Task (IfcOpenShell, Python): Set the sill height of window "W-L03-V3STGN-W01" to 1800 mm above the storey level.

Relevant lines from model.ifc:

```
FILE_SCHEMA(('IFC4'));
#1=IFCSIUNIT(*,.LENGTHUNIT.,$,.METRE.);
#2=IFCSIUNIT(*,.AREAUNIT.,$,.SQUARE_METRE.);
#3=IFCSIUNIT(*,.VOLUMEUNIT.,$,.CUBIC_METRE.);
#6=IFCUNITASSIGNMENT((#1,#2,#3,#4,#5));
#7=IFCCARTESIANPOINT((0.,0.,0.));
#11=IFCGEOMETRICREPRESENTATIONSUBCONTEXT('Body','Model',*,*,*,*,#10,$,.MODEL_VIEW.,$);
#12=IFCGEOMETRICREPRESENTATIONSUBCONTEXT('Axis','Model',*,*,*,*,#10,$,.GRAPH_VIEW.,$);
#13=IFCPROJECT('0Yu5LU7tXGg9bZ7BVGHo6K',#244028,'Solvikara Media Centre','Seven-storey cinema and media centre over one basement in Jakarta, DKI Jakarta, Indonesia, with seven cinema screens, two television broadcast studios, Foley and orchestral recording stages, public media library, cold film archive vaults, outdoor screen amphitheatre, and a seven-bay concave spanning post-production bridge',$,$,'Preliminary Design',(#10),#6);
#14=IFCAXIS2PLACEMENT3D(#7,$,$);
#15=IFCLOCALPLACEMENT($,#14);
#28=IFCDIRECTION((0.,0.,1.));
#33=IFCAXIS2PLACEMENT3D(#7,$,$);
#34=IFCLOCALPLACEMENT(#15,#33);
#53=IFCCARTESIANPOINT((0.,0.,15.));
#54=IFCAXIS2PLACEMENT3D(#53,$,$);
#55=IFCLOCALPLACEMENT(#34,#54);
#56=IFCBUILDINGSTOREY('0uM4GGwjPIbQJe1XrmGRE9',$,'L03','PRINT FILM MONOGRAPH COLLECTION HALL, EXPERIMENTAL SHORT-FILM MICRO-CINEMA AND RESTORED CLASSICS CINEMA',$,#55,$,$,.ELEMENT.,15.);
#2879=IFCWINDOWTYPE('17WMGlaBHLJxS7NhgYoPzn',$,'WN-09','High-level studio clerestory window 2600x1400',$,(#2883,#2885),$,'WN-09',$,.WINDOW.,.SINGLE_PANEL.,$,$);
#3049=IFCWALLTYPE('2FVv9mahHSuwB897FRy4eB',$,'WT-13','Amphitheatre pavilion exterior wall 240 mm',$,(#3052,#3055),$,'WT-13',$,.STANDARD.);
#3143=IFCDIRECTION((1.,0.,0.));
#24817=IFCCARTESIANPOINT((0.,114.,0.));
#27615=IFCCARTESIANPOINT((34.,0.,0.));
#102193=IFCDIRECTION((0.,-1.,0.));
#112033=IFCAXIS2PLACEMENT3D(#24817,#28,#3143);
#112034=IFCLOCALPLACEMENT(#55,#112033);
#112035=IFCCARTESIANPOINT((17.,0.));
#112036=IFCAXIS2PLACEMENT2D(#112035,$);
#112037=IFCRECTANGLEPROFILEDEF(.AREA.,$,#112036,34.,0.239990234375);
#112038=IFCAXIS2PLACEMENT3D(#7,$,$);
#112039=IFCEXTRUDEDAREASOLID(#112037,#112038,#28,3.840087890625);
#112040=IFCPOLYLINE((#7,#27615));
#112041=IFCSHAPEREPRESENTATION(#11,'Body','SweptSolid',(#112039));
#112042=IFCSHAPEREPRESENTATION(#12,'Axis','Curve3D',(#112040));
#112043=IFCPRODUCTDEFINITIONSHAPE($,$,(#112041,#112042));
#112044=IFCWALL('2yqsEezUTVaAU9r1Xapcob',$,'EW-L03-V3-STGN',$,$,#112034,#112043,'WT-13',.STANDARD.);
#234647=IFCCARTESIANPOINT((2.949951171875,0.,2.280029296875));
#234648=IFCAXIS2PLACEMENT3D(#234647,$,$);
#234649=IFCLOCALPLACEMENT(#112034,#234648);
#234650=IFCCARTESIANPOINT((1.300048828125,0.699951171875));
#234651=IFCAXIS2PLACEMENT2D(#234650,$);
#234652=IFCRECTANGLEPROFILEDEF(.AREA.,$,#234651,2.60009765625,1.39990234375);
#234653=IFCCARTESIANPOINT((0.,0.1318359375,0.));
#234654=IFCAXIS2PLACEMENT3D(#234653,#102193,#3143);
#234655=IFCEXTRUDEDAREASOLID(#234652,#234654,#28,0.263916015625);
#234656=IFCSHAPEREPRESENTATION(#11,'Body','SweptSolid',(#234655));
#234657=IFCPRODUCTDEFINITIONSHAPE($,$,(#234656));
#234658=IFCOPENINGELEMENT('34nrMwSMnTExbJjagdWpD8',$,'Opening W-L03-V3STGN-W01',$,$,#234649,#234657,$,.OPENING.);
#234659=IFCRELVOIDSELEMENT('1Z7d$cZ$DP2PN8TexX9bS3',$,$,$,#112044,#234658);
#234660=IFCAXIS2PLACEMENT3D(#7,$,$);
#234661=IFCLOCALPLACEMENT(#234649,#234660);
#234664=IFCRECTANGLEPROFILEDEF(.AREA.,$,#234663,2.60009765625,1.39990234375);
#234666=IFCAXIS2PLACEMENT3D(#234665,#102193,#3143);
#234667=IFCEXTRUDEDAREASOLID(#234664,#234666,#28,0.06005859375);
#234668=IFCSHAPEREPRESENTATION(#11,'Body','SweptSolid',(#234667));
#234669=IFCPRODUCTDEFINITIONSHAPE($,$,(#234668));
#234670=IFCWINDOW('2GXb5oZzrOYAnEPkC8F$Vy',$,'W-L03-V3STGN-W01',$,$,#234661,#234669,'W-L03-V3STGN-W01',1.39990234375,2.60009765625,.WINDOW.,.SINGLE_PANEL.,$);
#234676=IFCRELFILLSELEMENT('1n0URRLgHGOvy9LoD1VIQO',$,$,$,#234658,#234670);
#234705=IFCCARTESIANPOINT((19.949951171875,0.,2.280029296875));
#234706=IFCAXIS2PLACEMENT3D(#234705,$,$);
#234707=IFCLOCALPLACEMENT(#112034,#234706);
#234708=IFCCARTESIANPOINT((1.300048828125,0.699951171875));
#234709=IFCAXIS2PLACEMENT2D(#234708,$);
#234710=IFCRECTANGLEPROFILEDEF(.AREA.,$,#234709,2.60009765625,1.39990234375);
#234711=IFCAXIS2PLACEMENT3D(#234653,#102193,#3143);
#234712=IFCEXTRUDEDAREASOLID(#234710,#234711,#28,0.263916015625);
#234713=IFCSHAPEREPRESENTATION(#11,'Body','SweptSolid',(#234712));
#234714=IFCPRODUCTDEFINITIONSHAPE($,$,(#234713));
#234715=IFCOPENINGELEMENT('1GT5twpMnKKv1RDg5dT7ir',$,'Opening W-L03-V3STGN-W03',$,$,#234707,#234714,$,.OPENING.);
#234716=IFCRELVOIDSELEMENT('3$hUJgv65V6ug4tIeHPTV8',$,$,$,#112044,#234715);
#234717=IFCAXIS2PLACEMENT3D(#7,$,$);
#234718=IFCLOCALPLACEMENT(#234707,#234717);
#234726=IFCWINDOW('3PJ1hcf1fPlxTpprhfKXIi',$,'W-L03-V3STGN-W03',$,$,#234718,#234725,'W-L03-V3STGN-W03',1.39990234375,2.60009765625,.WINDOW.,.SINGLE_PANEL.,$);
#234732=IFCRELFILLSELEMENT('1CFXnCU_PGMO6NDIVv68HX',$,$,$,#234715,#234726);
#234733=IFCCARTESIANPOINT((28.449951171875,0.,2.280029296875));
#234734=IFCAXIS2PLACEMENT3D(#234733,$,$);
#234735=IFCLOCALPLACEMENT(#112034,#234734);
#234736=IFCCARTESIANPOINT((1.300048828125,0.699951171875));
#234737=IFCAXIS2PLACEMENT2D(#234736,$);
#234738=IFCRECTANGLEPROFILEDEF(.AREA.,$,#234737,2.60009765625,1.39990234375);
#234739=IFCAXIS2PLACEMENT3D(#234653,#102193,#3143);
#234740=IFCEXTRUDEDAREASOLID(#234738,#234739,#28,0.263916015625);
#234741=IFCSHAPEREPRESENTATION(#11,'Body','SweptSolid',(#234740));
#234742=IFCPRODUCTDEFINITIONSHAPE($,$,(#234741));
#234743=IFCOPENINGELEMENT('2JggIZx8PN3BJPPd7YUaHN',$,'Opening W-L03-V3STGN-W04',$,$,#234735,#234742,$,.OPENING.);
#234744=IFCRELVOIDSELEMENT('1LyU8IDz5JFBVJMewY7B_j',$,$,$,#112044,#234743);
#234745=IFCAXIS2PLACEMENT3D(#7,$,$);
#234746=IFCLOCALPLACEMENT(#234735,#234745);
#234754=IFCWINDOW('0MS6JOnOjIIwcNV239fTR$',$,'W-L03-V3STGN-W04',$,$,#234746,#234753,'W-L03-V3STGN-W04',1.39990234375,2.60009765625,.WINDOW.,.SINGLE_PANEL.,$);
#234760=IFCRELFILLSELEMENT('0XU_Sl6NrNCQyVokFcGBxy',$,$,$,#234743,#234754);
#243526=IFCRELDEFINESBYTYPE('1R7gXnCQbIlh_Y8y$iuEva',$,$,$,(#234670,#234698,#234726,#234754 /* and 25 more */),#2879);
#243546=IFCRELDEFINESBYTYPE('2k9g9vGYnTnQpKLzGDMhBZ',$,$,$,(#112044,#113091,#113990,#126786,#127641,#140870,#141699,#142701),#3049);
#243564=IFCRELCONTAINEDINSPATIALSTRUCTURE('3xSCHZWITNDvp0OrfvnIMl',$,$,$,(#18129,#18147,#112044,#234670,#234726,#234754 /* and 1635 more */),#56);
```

```python
import numpy as np
import ifcopenshell
import ifcopenshell.api.geometry
import ifcopenshell.geom
import ifcopenshell.util.element
import ifcopenshell.util.placement
import ifcopenshell.util.shape
import ifcopenshell.util.unit

model = ifcopenshell.open("model.ifc")
unit_scale = ifcopenshell.util.unit.calculate_unit_scale(model)

window = model.by_id(234670)
opening = window.FillsVoids[0].RelatingOpeningElement
storey = ifcopenshell.util.element.get_container(window, ifc_class="IfcBuildingStorey")
level = ifcopenshell.util.placement.get_local_placement(storey.ObjectPlacement)[2, 3]

# The opening's origin need not be at the sill, so measure its lowest point.
shape = ifcopenshell.geom.create_shape(ifcopenshell.geom.settings(), opening)
bottom = ifcopenshell.util.shape.get_shape_bottom_elevation(shape, shape.geometry) / unit_scale
dz = level + 1.8 - bottom

shift = np.array([0.0, 0.0, dz])
# The window is placed relative to its opening, so it follows when the opening moves.
matrix = ifcopenshell.util.placement.get_local_placement(opening.ObjectPlacement)
matrix[:3, 3] += shift
ifcopenshell.api.geometry.edit_object_placement(
    model, product=opening, matrix=matrix, is_si=False, should_transform_children=True
)

print(f"moved by {dz * unit_scale:+.3f} m")

model.write("model-out.ifc")
```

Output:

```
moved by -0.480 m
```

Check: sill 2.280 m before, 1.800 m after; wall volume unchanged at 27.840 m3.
